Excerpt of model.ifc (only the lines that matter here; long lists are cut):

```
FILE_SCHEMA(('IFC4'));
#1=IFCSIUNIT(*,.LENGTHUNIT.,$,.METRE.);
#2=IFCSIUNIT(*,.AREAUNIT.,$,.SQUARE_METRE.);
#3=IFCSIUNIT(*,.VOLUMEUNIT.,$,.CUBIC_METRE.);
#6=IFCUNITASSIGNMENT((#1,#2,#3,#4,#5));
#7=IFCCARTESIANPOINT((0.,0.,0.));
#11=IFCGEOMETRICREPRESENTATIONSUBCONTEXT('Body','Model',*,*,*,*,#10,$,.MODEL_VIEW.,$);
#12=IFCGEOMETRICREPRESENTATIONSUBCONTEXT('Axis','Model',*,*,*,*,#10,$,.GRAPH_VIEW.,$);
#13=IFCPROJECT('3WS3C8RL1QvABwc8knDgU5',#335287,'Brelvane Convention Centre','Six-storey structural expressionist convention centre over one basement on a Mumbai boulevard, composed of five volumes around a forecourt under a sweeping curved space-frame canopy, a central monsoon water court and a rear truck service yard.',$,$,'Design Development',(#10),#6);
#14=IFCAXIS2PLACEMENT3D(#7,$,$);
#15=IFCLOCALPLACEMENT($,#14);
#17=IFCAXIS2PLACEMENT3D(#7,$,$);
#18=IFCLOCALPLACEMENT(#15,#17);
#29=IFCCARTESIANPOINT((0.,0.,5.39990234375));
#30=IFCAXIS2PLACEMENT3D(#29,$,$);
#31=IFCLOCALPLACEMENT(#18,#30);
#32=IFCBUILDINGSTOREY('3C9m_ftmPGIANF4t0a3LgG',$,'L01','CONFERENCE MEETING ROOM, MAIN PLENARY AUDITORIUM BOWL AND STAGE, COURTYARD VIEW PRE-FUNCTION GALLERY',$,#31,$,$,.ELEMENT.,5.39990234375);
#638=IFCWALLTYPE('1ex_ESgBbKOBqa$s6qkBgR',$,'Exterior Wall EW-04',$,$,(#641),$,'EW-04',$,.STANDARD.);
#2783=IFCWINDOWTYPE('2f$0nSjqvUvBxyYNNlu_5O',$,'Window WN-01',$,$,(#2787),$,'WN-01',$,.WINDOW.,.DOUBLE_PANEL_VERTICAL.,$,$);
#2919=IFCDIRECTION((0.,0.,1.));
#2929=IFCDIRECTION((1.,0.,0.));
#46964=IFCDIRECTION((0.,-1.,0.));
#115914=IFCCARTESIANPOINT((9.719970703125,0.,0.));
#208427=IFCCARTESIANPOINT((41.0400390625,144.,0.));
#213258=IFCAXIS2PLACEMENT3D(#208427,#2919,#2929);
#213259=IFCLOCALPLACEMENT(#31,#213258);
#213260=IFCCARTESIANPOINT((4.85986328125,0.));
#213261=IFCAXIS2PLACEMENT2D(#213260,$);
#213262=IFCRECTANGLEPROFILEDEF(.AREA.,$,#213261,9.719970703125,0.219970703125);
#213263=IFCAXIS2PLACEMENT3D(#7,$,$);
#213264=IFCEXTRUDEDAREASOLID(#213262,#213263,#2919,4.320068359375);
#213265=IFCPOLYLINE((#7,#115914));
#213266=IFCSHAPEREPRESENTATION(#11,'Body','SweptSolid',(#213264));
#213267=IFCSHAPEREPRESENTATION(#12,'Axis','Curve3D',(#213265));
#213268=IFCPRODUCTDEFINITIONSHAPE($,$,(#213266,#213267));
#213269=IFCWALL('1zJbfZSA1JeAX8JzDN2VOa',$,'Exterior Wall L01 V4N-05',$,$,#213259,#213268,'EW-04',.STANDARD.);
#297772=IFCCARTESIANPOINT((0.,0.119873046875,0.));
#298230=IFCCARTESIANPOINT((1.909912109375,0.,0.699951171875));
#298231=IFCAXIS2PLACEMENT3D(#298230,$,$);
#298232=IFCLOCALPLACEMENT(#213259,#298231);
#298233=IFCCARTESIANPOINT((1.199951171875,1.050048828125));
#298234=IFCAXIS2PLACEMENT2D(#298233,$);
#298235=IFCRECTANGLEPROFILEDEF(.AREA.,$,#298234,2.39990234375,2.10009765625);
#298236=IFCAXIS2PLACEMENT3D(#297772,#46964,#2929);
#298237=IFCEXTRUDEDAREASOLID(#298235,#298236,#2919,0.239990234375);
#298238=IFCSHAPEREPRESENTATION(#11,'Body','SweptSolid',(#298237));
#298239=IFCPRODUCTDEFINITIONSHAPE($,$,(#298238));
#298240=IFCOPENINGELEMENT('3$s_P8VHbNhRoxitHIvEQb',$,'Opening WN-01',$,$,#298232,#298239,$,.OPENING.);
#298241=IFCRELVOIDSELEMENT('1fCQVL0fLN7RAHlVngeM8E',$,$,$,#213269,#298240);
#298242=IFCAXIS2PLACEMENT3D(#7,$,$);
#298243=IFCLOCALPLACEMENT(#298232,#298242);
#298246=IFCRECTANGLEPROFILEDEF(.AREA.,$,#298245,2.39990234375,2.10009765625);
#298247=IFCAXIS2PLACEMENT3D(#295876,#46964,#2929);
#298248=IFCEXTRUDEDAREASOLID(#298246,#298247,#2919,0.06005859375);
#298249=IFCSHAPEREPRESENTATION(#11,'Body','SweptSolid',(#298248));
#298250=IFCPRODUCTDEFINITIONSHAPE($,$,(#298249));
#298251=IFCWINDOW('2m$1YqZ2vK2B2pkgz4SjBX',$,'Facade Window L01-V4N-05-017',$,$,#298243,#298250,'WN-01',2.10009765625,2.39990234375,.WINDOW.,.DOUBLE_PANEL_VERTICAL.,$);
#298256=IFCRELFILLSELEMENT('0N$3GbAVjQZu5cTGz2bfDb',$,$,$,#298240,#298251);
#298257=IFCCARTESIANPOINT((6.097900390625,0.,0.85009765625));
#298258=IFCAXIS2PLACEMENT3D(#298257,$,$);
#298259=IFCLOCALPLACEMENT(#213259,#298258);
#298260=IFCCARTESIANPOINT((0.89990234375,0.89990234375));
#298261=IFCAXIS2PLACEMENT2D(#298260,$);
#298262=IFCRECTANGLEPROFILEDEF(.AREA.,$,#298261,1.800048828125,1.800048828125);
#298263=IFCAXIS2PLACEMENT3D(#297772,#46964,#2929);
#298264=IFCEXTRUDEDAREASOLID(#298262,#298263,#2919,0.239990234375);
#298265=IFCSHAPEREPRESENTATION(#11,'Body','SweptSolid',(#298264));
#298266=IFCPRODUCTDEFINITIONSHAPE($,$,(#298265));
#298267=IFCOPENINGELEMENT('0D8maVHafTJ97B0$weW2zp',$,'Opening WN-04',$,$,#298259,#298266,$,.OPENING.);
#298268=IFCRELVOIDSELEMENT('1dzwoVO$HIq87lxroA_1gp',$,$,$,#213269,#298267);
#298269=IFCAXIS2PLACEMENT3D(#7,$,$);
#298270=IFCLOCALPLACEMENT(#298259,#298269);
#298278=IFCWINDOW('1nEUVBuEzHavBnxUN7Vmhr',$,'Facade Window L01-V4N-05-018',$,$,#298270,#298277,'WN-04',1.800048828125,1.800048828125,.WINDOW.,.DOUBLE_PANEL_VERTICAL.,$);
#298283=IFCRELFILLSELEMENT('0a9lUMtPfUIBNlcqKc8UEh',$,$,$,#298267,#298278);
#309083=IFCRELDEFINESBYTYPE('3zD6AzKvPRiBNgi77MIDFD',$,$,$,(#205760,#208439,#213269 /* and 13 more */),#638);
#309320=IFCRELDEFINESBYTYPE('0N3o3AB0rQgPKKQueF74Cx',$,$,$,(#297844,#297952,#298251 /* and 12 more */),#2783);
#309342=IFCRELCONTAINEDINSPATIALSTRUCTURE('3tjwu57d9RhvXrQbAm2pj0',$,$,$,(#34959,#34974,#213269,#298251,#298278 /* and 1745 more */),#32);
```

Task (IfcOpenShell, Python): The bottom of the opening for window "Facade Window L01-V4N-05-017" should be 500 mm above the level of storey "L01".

```python
import numpy as np
import ifcopenshell
import ifcopenshell.api.geometry
import ifcopenshell.geom
import ifcopenshell.util.element
import ifcopenshell.util.placement
import ifcopenshell.util.shape
import ifcopenshell.util.unit

model = ifcopenshell.open("model.ifc")
unit_scale = ifcopenshell.util.unit.calculate_unit_scale(model)

window = model.by_guid("2m$1YqZ2vK2B2pkgz4SjBX")
opening = window.FillsVoids[0].RelatingOpeningElement
storey = ifcopenshell.util.element.get_container(window, ifc_class="IfcBuildingStorey")
level = ifcopenshell.util.placement.get_local_placement(storey.ObjectPlacement)[2, 3]

# The opening's origin need not be at the sill, so measure its lowest point.
shape = ifcopenshell.geom.create_shape(ifcopenshell.geom.settings(), opening)
bottom = ifcopenshell.util.shape.get_shape_bottom_elevation(shape, shape.geometry) / unit_scale
dz = level + 0.5 - bottom

shift = np.array([0.0, 0.0, dz])
# The window is placed relative to its opening, so it follows when the opening moves.
matrix = ifcopenshell.util.placement.get_local_placement(opening.ObjectPlacement)
matrix[:3, 3] += shift
ifcopenshell.api.geometry.edit_object_placement(
    model, product=opening, matrix=matrix, is_si=False, should_transform_children=True
)

print(f"moved by {dz * unit_scale:+.3f} m")

model.write("model_updated.ifc")
```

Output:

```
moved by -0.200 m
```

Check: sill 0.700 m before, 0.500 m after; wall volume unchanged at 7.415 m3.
